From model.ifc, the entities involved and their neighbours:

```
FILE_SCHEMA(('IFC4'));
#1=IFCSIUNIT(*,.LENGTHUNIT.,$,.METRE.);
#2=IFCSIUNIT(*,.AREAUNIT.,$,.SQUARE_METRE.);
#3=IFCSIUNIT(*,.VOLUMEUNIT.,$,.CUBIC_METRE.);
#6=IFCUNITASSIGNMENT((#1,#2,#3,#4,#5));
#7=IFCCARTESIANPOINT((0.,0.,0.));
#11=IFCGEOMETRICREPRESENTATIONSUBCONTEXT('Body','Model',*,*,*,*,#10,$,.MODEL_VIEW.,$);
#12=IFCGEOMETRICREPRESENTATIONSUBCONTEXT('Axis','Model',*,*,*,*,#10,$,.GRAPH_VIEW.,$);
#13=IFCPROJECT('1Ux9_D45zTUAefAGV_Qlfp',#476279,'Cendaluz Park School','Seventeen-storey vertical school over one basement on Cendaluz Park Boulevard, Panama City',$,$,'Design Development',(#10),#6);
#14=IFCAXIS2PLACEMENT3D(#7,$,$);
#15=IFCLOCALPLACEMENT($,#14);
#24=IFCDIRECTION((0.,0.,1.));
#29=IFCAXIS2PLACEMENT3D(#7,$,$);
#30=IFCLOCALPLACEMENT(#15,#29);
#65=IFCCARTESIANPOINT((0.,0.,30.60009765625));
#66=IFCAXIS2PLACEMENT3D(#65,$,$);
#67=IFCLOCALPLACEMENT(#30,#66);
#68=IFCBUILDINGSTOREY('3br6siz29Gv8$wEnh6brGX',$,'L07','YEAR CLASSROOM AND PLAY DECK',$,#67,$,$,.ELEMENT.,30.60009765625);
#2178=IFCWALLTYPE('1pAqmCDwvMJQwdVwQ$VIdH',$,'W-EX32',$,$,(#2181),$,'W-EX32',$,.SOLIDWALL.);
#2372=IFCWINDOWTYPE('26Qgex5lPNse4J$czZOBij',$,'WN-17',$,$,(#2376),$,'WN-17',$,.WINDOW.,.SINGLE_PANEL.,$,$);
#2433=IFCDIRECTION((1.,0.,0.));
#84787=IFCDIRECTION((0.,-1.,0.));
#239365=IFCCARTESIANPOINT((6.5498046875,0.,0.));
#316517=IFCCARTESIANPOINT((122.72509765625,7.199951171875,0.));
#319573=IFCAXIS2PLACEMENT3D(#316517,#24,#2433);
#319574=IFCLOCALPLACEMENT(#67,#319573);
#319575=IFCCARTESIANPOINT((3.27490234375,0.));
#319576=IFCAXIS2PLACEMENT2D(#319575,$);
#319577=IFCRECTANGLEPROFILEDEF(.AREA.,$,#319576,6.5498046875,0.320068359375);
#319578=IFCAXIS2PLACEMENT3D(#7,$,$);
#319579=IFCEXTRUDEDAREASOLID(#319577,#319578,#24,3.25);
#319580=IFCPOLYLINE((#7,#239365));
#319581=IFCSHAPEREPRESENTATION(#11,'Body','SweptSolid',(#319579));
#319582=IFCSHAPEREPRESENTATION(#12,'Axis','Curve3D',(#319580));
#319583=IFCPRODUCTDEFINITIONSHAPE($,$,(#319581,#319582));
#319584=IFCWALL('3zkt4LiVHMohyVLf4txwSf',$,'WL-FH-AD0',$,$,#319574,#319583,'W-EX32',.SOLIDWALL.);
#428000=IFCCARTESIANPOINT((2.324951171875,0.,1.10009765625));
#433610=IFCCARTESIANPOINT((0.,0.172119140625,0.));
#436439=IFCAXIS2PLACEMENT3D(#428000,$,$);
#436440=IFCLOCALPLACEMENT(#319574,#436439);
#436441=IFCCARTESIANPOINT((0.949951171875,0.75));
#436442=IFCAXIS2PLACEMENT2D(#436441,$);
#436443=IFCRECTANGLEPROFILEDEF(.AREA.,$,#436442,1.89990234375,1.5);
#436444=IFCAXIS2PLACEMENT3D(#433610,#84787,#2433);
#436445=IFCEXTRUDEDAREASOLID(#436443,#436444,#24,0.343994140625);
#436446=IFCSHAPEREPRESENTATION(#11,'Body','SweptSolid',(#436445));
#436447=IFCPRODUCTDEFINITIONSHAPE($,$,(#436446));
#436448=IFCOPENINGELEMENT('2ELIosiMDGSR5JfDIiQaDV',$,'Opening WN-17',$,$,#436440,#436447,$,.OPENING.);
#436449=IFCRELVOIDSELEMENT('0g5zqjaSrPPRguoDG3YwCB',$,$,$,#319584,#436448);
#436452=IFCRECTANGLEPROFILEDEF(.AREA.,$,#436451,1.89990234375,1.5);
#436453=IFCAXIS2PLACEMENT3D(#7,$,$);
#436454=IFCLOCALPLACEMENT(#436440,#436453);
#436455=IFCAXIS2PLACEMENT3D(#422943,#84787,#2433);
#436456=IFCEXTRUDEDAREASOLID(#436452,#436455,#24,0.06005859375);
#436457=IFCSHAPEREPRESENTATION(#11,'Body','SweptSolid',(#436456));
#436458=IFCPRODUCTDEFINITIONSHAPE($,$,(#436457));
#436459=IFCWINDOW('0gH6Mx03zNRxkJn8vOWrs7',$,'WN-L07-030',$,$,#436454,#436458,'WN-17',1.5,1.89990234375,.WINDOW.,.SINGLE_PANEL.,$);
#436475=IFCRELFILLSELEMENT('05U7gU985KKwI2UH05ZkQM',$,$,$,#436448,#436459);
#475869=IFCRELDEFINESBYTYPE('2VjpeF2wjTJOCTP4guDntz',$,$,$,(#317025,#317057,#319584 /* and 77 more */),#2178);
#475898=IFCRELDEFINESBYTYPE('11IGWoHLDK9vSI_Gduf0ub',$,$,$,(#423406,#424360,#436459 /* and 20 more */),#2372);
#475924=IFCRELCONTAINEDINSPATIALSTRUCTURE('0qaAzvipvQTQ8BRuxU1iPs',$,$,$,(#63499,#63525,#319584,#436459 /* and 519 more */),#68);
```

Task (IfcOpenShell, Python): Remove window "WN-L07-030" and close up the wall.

```python
import ifcopenshell
import ifcopenshell.api.feature
import ifcopenshell.api.root
import ifcopenshell.geom
import ifcopenshell.util.shape

model = ifcopenshell.open("model.ifc")
settings = ifcopenshell.geom.settings()


def volume(element):
    """Net volume in cubic metres, openings subtracted."""
    shape = ifcopenshell.geom.create_shape(settings, element)
    return ifcopenshell.util.shape.get_volume(shape.geometry)


window = model.by_guid("0gH6Mx03zNRxkJn8vOWrs7")
opening = window.FillsVoids[0].RelatingOpeningElement
wall = opening.VoidsElements[0].RelatingBuildingElement
before = volume(wall)

ifcopenshell.api.root.remove_product(model, product=window)
ifcopenshell.api.feature.remove_feature(model, feature=opening)

after = volume(wall)

print(f"wall volume {before:.3f} -> {after:.3f} m3")

model.write("model-out.ifc")
```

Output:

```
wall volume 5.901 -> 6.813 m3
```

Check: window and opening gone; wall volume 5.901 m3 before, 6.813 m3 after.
